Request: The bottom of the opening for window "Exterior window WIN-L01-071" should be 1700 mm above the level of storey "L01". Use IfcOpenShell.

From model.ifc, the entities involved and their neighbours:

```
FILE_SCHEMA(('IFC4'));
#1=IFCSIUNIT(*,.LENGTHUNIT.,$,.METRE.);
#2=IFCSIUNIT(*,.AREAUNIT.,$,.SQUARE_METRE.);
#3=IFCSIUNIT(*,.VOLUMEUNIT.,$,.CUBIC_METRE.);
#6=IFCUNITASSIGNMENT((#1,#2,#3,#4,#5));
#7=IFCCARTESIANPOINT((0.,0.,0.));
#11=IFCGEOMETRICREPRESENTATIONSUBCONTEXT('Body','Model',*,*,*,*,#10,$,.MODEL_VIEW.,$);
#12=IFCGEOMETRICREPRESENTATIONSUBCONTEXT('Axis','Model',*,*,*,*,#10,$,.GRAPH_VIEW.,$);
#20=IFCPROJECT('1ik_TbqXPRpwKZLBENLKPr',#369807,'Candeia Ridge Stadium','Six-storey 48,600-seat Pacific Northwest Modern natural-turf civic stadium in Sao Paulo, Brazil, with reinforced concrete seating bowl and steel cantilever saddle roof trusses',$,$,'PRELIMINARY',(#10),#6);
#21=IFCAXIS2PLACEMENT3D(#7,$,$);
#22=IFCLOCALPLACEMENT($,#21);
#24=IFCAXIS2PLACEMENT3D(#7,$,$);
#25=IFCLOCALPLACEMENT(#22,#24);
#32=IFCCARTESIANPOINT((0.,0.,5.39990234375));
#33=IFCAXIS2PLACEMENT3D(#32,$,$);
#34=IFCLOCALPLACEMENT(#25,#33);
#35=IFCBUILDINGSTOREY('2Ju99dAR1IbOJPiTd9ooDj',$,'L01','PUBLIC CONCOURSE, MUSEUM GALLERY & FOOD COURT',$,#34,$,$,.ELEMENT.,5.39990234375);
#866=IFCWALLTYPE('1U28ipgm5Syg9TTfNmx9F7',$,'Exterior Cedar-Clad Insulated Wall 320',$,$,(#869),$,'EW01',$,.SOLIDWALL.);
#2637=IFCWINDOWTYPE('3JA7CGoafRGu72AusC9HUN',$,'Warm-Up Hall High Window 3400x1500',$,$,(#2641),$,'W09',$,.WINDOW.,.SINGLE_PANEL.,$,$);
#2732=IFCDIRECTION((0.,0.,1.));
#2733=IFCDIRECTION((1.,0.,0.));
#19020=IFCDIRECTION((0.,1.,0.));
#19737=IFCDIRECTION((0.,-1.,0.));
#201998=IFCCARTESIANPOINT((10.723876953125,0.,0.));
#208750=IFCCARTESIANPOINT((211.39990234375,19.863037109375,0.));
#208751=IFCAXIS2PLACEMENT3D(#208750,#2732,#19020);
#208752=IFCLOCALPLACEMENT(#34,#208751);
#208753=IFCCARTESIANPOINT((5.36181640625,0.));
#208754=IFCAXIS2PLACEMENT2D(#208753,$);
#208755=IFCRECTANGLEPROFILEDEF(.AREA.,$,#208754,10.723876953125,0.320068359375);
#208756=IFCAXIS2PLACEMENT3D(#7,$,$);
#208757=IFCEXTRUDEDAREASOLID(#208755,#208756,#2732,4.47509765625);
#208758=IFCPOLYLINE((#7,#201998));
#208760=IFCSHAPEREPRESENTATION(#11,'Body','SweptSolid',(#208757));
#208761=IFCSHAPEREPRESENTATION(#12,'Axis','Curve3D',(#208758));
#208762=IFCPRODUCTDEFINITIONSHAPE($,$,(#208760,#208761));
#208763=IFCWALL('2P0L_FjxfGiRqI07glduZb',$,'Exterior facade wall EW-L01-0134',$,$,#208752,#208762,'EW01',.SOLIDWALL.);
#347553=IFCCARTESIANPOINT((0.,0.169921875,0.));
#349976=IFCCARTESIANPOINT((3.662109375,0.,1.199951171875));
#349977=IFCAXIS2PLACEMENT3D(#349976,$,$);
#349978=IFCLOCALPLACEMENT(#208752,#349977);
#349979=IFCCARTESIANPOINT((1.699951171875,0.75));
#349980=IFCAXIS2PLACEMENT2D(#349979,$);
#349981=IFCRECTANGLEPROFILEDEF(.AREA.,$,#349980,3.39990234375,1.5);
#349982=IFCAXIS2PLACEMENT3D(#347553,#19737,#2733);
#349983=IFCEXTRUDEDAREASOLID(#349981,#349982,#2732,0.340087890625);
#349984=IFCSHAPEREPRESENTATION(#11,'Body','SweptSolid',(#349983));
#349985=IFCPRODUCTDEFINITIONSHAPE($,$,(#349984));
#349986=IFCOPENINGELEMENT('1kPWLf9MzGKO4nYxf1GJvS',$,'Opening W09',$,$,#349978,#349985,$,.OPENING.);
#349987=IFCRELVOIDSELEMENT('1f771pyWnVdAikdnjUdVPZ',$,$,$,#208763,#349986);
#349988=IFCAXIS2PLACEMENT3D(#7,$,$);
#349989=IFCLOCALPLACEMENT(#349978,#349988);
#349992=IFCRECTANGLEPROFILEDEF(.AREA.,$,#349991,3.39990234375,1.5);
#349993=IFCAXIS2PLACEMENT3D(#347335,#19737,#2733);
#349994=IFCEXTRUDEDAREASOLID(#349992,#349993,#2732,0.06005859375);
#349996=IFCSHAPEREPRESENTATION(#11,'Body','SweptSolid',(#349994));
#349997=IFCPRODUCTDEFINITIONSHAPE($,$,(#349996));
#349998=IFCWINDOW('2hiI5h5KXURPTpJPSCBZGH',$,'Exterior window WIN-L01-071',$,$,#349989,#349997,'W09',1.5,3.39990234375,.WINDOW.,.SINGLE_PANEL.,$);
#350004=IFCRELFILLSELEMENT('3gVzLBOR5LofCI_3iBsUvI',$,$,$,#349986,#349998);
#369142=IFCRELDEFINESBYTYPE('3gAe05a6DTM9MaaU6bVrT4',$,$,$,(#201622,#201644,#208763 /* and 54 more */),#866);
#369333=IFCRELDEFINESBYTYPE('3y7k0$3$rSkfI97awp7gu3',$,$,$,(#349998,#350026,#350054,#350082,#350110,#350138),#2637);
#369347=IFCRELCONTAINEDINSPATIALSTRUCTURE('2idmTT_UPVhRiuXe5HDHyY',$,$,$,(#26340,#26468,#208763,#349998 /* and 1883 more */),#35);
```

```python
import numpy as np
import ifcopenshell
import ifcopenshell.api.geometry
import ifcopenshell.geom
import ifcopenshell.util.element
import ifcopenshell.util.placement
import ifcopenshell.util.shape
import ifcopenshell.util.unit

model = ifcopenshell.open("model.ifc")
unit_scale = ifcopenshell.util.unit.calculate_unit_scale(model)

window = model.by_guid("2hiI5h5KXURPTpJPSCBZGH")
opening = window.FillsVoids[0].RelatingOpeningElement
storey = ifcopenshell.util.element.get_container(window, ifc_class="IfcBuildingStorey")
level = ifcopenshell.util.placement.get_local_placement(storey.ObjectPlacement)[2, 3]

# The opening's origin need not be at the sill, so measure its lowest point.
shape = ifcopenshell.geom.create_shape(ifcopenshell.geom.settings(), opening)
bottom = ifcopenshell.util.shape.get_shape_bottom_elevation(shape, shape.geometry) / unit_scale
dz = level + 1.7 / unit_scale - bottom

shift = np.array([0.0, 0.0, dz])
# The window is placed relative to its opening, so it follows when the opening moves.
matrix = ifcopenshell.util.placement.get_local_placement(opening.ObjectPlacement)
matrix[:3, 3] += shift
ifcopenshell.api.geometry.edit_object_placement(
    model, product=opening, matrix=matrix, is_si=False, should_transform_children=True
)

print(f"moved by {dz * unit_scale:+.3f} m")

model.write("model_rev.ifc")
```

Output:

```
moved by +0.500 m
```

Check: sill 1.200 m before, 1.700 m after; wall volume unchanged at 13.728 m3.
